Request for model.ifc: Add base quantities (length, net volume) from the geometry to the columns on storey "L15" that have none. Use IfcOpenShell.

First a look at what the model holds.

```python
import ifcopenshell
import ifcopenshell.util.element
import ifcopenshell.util.unit

model = ifcopenshell.open("model.ifc")
print(model.schema)
for unit_type in ("LENGTHUNIT", "AREAUNIT", "VOLUMEUNIT"):
    print(unit_type, ifcopenshell.util.unit.calculate_unit_scale(model, unit_type))
storey = next(s for s in model.by_type("IfcBuildingStorey") if s.Name == "L15")
columns = [e for e in ifcopenshell.util.element.get_decomposition(storey) if e.is_a("IfcColumn")]
for e in sorted(columns, key=lambda e: e.id()):
    print(e.id(), e.is_a(), e.Name, list(ifcopenshell.util.element.get_psets(e, qtos_only=True)), sep=" | ")
```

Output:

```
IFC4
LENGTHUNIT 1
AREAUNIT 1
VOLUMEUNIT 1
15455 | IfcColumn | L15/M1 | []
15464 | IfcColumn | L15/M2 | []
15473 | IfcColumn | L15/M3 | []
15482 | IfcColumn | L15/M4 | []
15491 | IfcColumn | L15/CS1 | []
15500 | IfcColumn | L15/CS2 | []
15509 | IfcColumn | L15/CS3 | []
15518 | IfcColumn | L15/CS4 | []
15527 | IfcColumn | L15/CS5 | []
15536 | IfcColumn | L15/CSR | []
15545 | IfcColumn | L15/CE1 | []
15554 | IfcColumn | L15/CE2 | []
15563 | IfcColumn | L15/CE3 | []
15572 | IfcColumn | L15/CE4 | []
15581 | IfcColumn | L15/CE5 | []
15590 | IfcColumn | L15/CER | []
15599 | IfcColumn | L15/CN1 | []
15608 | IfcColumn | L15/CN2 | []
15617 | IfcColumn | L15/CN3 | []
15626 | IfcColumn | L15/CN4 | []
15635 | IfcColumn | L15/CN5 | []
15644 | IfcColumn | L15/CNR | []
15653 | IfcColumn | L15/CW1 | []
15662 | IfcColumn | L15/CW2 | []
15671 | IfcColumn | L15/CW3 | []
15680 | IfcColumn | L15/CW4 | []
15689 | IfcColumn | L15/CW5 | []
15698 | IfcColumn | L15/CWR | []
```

```python
import ifcopenshell
import ifcopenshell.api.pset
import ifcopenshell.geom
import ifcopenshell.util.element
import ifcopenshell.util.shape
import ifcopenshell.util.unit

model = ifcopenshell.open("model.ifc")
unit_scale = ifcopenshell.util.unit.calculate_unit_scale(model)
volume_scale = ifcopenshell.util.unit.calculate_unit_scale(model, "VOLUMEUNIT")
settings = ifcopenshell.geom.settings()

storey = next(s for s in model.by_type("IfcBuildingStorey") if s.Name == "L15")
columns = [e for e in ifcopenshell.util.element.get_decomposition(storey) if e.is_a("IfcColumn")]

for e in sorted(columns, key=lambda e: e.id()):
    if ifcopenshell.util.element.get_psets(e, qtos_only=True, should_inherit=False):
        continue
    # Geometry comes back in metres, in the element's own axes.
    shape = ifcopenshell.geom.create_shape(settings, e)
    values = {
        "Length": ifcopenshell.util.shape.get_z(shape.geometry) / unit_scale,
        "NetVolume": ifcopenshell.util.shape.get_volume(shape.geometry) / volume_scale,
    }
    qto = ifcopenshell.api.pset.add_qto(model, product=e, name="Qto_ColumnBaseQuantities")
    ifcopenshell.api.pset.edit_qto(model, qto=qto, properties=values)
    print(e.id(), {k: round(v, 3) for k, v in values.items()})

model.write("model_edited.ifc")
```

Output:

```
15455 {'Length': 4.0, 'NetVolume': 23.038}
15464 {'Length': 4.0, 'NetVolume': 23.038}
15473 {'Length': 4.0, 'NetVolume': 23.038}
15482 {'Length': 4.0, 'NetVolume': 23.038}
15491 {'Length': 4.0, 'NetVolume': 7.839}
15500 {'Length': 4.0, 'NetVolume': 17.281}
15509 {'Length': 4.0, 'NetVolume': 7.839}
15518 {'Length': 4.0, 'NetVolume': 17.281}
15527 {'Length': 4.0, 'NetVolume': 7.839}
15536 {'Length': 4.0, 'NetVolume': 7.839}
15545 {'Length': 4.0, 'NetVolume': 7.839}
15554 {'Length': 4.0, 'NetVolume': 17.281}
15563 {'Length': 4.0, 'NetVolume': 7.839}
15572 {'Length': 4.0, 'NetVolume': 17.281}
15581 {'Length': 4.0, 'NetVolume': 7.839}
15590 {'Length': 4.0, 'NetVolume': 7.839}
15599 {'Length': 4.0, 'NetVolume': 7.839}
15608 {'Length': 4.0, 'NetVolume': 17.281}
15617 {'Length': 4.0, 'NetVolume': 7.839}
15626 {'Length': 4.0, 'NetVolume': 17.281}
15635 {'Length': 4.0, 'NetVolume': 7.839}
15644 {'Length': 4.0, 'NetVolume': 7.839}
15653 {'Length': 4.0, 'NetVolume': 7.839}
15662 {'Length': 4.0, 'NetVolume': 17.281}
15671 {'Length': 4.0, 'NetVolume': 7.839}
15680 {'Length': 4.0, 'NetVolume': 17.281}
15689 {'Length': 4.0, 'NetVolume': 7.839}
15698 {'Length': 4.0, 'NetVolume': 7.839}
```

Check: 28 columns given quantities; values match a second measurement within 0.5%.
